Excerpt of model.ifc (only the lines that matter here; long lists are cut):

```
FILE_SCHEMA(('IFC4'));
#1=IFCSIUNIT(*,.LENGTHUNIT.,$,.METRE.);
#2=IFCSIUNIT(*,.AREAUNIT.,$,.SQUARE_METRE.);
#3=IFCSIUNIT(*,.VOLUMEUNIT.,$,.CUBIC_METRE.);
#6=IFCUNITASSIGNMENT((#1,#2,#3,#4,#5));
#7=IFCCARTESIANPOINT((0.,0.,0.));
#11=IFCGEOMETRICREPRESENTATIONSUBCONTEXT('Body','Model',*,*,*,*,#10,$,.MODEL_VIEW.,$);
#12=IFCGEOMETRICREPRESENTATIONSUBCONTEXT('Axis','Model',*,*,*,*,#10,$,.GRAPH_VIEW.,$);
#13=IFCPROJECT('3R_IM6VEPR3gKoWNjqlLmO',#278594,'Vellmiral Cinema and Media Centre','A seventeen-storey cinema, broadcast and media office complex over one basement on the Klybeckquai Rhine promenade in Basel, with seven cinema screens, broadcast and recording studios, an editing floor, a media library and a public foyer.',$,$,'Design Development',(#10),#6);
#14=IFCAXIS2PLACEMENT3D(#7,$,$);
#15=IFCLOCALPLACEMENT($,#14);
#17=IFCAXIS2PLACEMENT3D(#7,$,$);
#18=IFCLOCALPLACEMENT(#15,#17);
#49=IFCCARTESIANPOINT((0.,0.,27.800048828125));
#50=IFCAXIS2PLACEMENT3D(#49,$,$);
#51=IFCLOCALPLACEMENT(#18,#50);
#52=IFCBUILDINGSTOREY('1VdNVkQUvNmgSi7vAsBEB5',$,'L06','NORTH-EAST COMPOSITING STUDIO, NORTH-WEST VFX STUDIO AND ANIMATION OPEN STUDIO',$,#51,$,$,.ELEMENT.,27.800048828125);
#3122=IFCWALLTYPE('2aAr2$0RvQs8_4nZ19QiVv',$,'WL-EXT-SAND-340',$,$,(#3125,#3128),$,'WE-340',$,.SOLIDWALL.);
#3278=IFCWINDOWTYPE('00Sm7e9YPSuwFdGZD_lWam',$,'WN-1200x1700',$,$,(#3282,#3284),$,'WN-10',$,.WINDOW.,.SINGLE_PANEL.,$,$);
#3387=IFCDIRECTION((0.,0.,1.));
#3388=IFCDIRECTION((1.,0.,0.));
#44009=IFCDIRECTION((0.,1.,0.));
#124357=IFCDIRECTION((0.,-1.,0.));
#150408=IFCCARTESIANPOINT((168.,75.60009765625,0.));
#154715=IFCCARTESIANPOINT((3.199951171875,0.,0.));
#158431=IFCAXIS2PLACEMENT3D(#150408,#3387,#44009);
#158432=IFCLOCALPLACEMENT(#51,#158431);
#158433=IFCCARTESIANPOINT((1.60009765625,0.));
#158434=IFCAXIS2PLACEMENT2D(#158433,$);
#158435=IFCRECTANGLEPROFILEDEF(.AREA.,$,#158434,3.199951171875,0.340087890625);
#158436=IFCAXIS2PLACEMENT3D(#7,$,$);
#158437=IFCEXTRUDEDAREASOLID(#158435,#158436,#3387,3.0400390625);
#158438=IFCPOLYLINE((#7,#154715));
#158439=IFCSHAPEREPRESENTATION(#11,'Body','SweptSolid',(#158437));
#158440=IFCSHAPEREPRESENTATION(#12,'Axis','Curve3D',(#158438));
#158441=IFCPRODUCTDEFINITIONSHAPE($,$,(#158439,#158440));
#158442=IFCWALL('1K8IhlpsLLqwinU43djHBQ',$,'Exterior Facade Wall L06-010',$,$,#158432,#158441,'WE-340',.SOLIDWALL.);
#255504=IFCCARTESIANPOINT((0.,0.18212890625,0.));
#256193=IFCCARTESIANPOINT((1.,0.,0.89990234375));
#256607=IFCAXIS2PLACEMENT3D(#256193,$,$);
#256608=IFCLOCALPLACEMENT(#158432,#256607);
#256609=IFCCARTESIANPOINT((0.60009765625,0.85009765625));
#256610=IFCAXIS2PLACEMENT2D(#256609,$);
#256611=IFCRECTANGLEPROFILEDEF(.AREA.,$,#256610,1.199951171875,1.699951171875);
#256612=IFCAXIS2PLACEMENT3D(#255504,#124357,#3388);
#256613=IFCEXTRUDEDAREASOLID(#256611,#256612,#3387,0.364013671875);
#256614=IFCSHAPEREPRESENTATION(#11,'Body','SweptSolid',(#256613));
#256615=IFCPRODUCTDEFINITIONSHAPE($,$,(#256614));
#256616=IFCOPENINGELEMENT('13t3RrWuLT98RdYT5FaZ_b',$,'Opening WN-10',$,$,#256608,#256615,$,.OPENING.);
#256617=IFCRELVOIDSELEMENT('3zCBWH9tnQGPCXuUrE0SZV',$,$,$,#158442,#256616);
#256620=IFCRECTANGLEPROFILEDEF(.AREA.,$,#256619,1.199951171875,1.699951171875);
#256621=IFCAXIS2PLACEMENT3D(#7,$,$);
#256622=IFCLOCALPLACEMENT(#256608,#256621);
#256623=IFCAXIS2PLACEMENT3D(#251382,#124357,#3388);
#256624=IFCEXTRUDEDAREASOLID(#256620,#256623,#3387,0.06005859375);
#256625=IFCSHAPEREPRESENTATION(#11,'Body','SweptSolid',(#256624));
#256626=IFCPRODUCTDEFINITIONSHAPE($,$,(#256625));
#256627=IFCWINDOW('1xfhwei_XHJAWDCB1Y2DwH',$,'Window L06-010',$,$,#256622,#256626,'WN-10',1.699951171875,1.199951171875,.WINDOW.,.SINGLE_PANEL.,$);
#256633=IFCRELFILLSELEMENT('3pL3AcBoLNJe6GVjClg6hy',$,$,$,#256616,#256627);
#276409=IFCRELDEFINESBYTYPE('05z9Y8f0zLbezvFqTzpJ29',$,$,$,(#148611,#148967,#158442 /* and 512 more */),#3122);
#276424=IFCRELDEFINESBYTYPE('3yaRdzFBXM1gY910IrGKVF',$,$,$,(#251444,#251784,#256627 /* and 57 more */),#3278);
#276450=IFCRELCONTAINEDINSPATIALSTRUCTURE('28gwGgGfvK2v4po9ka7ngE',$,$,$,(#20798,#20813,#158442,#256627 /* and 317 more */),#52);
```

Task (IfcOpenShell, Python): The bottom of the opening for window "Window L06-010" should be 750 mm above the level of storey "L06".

```python
import numpy as np
import ifcopenshell
import ifcopenshell.api.geometry
import ifcopenshell.geom
import ifcopenshell.util.element
import ifcopenshell.util.placement
import ifcopenshell.util.shape
import ifcopenshell.util.unit

model = ifcopenshell.open("model.ifc")
unit_scale = ifcopenshell.util.unit.calculate_unit_scale(model)

window = model.by_id(256627)
opening = window.FillsVoids[0].RelatingOpeningElement
storey = ifcopenshell.util.element.get_container(window, ifc_class="IfcBuildingStorey")
level = ifcopenshell.util.placement.get_local_placement(storey.ObjectPlacement)[2, 3]

# The opening's origin need not be at the sill, so measure its lowest point.
shape = ifcopenshell.geom.create_shape(ifcopenshell.geom.settings(), opening)
bottom = ifcopenshell.util.shape.get_shape_bottom_elevation(shape, shape.geometry) / unit_scale
dz = level + 0.75 / unit_scale - bottom

shift = np.array([0.0, 0.0, dz])
# The window is placed relative to its opening, so it follows when the opening moves.
matrix = ifcopenshell.util.placement.get_local_placement(opening.ObjectPlacement)
matrix[:3, 3] += shift
ifcopenshell.api.geometry.edit_object_placement(
    model, product=opening, matrix=matrix, is_si=False, should_transform_children=True
)

print(f"moved by {dz * unit_scale:+.3f} m")

model.write("model-out.ifc")
```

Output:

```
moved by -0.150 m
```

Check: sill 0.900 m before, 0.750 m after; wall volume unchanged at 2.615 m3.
